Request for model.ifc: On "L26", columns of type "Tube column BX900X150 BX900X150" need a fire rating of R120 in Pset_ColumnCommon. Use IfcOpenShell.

First a look at what the model holds.

```python
import ifcopenshell
import ifcopenshell.util.element

model = ifcopenshell.open("model.ifc")
print(model.schema)
storey = next(s for s in model.by_type("IfcBuildingStorey") if s.Name == "L26")
columns = [e for e in ifcopenshell.util.element.get_decomposition(storey) if e.is_a("IfcColumn")]
seen = {}
for e in columns:
    element_type = ifcopenshell.util.element.get_type(e)
    key = (element_type.Name if element_type != e and element_type else None, ifcopenshell.util.element.get_pset(e, "Pset_ColumnCommon", "FireRating"))
    seen[key] = seen.get(key, 0) + 1
for (name, value), count in sorted(seen.items(), key=str):
    print(count, "x", name, "|", value)
```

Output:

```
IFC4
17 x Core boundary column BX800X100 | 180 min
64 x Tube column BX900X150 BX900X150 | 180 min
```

```python
import ifcopenshell
import ifcopenshell.api.pset
import ifcopenshell.util.element

model = ifcopenshell.open("model.ifc")

storey = next(s for s in model.by_type("IfcBuildingStorey") if s.Name == "L26")
columns = [e for e in ifcopenshell.util.element.get_decomposition(storey) if e.is_a("IfcColumn")]

count = 0
for e in columns:
    element_type = ifcopenshell.util.element.get_type(e)
    if element_type in (None, e) or element_type.Name != "Tube column BX900X150 BX900X150":
        continue
    found = ifcopenshell.util.element.get_pset(e, "Pset_ColumnCommon", should_inherit=False)
    if found:
        pset = model.by_id(found["id"])
        if len(ifcopenshell.util.element.get_elements_by_pset(pset)) > 1:
            pset = ifcopenshell.api.pset.unshare_pset(model, products=[e], pset=pset)[0]
    else:
        pset = ifcopenshell.api.pset.add_pset(model, product=e, name="Pset_ColumnCommon")
    ifcopenshell.api.pset.edit_pset(model, pset=pset, properties={"FireRating": "R120"})
    count += 1

print(count, "columns updated")

model.write("model_updated.ifc")
```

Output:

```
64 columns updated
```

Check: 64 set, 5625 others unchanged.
